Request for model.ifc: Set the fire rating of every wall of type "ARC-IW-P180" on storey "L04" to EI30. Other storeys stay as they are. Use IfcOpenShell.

First a look at what the model holds.

```python
import ifcopenshell
import ifcopenshell.util.element

model = ifcopenshell.open("model.ifc")
print(model.schema)
storey = next(s for s in model.by_type("IfcBuildingStorey") if s.Name == "L04")
walls = [e for e in ifcopenshell.util.element.get_decomposition(storey) if e.is_a("IfcWall")]
seen = {}
for e in walls:
    element_type = ifcopenshell.util.element.get_type(e)
    key = (element_type.Name if element_type != e and element_type else None, ifcopenshell.util.element.get_pset(e, "Pset_WallCommon", "FireRating"))
    seen[key] = seen.get(key, 0) + 1
for (name, value), count in sorted(seen.items(), key=str):
    print(count, "x", name, "|", value)
```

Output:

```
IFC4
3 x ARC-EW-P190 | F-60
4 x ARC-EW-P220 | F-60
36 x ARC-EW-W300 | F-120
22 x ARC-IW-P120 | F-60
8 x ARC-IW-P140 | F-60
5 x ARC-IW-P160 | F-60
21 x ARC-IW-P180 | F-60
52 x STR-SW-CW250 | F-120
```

```python
import ifcopenshell
import ifcopenshell.api.pset
import ifcopenshell.util.element

model = ifcopenshell.open("model.ifc")

storey = next(s for s in model.by_type("IfcBuildingStorey") if s.Name == "L04")
walls = [e for e in ifcopenshell.util.element.get_decomposition(storey) if e.is_a("IfcWall")]

count = 0
for e in walls:
    element_type = ifcopenshell.util.element.get_type(e)
    if element_type in (None, e) or element_type.Name != "ARC-IW-P180":
        continue
    # add_pset returns the element's existing set when there is one.
    pset = ifcopenshell.api.pset.add_pset(model, product=e, name="Pset_WallCommon")
    ifcopenshell.api.pset.edit_pset(model, pset=pset, properties={"FireRating": "EI30"})
    count += 1

print(count, "walls updated")

model.write("model_v2.ifc")
```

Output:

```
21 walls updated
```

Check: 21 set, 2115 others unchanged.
